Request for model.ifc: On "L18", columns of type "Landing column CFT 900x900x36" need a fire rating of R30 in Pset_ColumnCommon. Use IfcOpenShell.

First a look at what the model holds.

```python
import ifcopenshell
import ifcopenshell.util.element

model = ifcopenshell.open("model.ifc")
print(model.schema)
storey = next(s for s in model.by_type("IfcBuildingStorey") if s.Name == "L18")
columns = [e for e in ifcopenshell.util.element.get_decomposition(storey) if e.is_a("IfcColumn")]
seen = {}
for e in columns:
    element_type = ifcopenshell.util.element.get_type(e)
    key = (element_type.Name if element_type != e and element_type else None, ifcopenshell.util.element.get_pset(e, "Pset_ColumnCommon", "FireRating"))
    seen[key] = seen.get(key, 0) + 1
for (name, value), count in sorted(seen.items(), key=str):
    print(count, "x", name, "|", value)
```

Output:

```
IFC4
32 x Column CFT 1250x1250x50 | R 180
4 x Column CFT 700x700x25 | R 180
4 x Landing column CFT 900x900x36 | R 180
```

```python
import ifcopenshell
import ifcopenshell.api.pset
import ifcopenshell.util.element

model = ifcopenshell.open("model.ifc")

storey = next(s for s in model.by_type("IfcBuildingStorey") if s.Name == "L18")
columns = [e for e in ifcopenshell.util.element.get_decomposition(storey) if e.is_a("IfcColumn")]

count = 0
for e in columns:
    element_type = ifcopenshell.util.element.get_type(e)
    if element_type in (None, e) or element_type.Name != "Landing column CFT 900x900x36":
        continue
    found = ifcopenshell.util.element.get_pset(e, "Pset_ColumnCommon", should_inherit=False)
    if found:
        pset = model.by_id(found["id"])
        if len(ifcopenshell.util.element.get_elements_by_pset(pset)) > 1:
            pset = ifcopenshell.api.pset.unshare_pset(model, products=[e], pset=pset)[0]
    else:
        pset = ifcopenshell.api.pset.add_pset(model, product=e, name="Pset_ColumnCommon")
    ifcopenshell.api.pset.edit_pset(model, pset=pset, properties={"FireRating": "R30"})
    count += 1

print(count, "columns updated")

model.write("model_updated.ifc")
```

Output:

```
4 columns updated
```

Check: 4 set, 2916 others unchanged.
